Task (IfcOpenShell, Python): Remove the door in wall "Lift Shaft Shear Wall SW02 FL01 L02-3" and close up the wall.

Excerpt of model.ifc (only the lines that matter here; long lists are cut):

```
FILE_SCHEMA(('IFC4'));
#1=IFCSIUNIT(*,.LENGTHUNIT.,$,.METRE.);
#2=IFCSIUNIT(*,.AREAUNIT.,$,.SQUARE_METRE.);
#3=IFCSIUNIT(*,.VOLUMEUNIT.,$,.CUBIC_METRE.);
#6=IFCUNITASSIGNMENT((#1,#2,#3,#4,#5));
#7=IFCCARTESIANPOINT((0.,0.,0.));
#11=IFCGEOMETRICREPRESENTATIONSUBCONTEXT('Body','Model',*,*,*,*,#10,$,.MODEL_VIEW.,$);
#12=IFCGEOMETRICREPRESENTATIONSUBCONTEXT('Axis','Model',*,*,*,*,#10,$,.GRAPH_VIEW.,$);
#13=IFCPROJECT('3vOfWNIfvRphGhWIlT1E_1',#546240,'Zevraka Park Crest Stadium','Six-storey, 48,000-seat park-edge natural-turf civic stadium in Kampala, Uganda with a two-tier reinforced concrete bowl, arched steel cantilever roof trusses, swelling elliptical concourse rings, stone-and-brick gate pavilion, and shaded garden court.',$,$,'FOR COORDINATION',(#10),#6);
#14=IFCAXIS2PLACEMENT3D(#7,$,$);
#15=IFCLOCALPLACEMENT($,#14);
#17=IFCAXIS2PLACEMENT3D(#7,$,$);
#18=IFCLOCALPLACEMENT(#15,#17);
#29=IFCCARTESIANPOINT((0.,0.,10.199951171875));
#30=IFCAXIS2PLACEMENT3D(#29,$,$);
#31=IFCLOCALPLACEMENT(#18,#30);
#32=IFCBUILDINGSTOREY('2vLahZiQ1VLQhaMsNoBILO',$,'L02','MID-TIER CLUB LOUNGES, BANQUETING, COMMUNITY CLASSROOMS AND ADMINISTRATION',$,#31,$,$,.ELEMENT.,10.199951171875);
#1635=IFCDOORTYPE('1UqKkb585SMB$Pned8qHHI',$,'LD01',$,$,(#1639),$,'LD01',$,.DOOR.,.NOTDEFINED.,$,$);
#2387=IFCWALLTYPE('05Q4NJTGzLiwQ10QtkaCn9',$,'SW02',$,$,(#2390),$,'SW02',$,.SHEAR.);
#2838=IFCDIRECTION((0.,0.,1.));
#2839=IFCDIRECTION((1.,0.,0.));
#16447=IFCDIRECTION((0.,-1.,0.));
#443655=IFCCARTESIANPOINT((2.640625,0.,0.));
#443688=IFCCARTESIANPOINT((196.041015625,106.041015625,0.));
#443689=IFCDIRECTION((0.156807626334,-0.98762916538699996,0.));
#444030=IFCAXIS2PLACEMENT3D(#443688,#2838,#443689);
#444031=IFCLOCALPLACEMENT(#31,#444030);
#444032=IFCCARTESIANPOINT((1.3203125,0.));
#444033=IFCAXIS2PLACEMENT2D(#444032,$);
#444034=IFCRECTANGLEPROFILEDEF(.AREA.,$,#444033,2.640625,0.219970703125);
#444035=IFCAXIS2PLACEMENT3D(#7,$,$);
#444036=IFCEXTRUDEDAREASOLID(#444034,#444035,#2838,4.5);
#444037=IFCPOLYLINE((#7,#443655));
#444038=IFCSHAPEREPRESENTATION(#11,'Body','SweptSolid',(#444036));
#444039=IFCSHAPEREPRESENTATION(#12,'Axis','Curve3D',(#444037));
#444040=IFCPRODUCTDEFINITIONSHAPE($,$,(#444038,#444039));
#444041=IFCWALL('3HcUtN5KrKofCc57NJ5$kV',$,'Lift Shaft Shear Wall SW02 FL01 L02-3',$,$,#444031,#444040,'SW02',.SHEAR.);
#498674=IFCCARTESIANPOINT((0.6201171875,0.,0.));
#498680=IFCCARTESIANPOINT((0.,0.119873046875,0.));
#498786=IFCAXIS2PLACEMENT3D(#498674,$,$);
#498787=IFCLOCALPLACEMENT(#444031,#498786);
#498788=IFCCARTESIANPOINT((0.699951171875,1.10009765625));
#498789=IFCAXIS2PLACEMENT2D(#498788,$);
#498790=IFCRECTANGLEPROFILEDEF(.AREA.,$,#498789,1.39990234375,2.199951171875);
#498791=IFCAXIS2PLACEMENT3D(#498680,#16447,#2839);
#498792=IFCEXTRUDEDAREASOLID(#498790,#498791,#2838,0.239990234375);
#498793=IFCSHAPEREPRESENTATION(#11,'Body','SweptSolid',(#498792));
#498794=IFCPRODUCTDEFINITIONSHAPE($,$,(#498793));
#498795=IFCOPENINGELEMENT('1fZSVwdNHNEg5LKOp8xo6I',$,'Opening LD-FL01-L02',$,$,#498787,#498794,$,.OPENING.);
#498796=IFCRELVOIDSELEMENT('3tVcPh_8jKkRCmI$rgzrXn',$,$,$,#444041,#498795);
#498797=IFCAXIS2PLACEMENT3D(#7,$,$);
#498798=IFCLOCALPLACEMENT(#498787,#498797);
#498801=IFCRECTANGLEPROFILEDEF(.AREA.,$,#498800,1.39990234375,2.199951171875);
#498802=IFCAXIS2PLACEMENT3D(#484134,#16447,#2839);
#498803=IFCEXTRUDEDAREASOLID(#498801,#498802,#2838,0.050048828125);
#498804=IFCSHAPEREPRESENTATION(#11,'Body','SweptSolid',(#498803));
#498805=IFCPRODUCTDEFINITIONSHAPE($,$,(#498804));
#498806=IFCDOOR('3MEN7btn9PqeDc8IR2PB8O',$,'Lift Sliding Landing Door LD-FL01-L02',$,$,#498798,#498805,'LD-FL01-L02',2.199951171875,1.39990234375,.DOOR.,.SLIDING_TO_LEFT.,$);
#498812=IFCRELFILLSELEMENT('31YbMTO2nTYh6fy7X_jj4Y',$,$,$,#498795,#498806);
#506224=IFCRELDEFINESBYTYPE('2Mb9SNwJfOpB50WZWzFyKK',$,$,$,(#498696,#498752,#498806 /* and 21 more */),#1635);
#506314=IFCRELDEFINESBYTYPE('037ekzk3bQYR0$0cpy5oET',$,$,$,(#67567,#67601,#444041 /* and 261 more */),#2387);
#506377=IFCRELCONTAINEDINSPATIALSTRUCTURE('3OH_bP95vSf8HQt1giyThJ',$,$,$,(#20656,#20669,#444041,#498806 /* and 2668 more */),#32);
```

```python
import ifcopenshell
import ifcopenshell.api.feature
import ifcopenshell.api.root
import ifcopenshell.geom
import ifcopenshell.util.shape

model = ifcopenshell.open("model.ifc")
settings = ifcopenshell.geom.settings()


def volume(element):
    """Net volume in cubic metres, openings subtracted."""
    shape = ifcopenshell.geom.create_shape(settings, element)
    return ifcopenshell.util.shape.get_volume(shape.geometry)


door = model.by_guid("3MEN7btn9PqeDc8IR2PB8O")
opening = door.FillsVoids[0].RelatingOpeningElement
wall = opening.VoidsElements[0].RelatingBuildingElement
before = volume(wall)

ifcopenshell.api.root.remove_product(model, product=door)
ifcopenshell.api.feature.remove_feature(model, feature=opening)

after = volume(wall)

print(f"wall volume {before:.3f} -> {after:.3f} m3")

model.write("model_v2.ifc")
```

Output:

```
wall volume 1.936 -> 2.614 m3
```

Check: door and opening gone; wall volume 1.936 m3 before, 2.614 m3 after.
